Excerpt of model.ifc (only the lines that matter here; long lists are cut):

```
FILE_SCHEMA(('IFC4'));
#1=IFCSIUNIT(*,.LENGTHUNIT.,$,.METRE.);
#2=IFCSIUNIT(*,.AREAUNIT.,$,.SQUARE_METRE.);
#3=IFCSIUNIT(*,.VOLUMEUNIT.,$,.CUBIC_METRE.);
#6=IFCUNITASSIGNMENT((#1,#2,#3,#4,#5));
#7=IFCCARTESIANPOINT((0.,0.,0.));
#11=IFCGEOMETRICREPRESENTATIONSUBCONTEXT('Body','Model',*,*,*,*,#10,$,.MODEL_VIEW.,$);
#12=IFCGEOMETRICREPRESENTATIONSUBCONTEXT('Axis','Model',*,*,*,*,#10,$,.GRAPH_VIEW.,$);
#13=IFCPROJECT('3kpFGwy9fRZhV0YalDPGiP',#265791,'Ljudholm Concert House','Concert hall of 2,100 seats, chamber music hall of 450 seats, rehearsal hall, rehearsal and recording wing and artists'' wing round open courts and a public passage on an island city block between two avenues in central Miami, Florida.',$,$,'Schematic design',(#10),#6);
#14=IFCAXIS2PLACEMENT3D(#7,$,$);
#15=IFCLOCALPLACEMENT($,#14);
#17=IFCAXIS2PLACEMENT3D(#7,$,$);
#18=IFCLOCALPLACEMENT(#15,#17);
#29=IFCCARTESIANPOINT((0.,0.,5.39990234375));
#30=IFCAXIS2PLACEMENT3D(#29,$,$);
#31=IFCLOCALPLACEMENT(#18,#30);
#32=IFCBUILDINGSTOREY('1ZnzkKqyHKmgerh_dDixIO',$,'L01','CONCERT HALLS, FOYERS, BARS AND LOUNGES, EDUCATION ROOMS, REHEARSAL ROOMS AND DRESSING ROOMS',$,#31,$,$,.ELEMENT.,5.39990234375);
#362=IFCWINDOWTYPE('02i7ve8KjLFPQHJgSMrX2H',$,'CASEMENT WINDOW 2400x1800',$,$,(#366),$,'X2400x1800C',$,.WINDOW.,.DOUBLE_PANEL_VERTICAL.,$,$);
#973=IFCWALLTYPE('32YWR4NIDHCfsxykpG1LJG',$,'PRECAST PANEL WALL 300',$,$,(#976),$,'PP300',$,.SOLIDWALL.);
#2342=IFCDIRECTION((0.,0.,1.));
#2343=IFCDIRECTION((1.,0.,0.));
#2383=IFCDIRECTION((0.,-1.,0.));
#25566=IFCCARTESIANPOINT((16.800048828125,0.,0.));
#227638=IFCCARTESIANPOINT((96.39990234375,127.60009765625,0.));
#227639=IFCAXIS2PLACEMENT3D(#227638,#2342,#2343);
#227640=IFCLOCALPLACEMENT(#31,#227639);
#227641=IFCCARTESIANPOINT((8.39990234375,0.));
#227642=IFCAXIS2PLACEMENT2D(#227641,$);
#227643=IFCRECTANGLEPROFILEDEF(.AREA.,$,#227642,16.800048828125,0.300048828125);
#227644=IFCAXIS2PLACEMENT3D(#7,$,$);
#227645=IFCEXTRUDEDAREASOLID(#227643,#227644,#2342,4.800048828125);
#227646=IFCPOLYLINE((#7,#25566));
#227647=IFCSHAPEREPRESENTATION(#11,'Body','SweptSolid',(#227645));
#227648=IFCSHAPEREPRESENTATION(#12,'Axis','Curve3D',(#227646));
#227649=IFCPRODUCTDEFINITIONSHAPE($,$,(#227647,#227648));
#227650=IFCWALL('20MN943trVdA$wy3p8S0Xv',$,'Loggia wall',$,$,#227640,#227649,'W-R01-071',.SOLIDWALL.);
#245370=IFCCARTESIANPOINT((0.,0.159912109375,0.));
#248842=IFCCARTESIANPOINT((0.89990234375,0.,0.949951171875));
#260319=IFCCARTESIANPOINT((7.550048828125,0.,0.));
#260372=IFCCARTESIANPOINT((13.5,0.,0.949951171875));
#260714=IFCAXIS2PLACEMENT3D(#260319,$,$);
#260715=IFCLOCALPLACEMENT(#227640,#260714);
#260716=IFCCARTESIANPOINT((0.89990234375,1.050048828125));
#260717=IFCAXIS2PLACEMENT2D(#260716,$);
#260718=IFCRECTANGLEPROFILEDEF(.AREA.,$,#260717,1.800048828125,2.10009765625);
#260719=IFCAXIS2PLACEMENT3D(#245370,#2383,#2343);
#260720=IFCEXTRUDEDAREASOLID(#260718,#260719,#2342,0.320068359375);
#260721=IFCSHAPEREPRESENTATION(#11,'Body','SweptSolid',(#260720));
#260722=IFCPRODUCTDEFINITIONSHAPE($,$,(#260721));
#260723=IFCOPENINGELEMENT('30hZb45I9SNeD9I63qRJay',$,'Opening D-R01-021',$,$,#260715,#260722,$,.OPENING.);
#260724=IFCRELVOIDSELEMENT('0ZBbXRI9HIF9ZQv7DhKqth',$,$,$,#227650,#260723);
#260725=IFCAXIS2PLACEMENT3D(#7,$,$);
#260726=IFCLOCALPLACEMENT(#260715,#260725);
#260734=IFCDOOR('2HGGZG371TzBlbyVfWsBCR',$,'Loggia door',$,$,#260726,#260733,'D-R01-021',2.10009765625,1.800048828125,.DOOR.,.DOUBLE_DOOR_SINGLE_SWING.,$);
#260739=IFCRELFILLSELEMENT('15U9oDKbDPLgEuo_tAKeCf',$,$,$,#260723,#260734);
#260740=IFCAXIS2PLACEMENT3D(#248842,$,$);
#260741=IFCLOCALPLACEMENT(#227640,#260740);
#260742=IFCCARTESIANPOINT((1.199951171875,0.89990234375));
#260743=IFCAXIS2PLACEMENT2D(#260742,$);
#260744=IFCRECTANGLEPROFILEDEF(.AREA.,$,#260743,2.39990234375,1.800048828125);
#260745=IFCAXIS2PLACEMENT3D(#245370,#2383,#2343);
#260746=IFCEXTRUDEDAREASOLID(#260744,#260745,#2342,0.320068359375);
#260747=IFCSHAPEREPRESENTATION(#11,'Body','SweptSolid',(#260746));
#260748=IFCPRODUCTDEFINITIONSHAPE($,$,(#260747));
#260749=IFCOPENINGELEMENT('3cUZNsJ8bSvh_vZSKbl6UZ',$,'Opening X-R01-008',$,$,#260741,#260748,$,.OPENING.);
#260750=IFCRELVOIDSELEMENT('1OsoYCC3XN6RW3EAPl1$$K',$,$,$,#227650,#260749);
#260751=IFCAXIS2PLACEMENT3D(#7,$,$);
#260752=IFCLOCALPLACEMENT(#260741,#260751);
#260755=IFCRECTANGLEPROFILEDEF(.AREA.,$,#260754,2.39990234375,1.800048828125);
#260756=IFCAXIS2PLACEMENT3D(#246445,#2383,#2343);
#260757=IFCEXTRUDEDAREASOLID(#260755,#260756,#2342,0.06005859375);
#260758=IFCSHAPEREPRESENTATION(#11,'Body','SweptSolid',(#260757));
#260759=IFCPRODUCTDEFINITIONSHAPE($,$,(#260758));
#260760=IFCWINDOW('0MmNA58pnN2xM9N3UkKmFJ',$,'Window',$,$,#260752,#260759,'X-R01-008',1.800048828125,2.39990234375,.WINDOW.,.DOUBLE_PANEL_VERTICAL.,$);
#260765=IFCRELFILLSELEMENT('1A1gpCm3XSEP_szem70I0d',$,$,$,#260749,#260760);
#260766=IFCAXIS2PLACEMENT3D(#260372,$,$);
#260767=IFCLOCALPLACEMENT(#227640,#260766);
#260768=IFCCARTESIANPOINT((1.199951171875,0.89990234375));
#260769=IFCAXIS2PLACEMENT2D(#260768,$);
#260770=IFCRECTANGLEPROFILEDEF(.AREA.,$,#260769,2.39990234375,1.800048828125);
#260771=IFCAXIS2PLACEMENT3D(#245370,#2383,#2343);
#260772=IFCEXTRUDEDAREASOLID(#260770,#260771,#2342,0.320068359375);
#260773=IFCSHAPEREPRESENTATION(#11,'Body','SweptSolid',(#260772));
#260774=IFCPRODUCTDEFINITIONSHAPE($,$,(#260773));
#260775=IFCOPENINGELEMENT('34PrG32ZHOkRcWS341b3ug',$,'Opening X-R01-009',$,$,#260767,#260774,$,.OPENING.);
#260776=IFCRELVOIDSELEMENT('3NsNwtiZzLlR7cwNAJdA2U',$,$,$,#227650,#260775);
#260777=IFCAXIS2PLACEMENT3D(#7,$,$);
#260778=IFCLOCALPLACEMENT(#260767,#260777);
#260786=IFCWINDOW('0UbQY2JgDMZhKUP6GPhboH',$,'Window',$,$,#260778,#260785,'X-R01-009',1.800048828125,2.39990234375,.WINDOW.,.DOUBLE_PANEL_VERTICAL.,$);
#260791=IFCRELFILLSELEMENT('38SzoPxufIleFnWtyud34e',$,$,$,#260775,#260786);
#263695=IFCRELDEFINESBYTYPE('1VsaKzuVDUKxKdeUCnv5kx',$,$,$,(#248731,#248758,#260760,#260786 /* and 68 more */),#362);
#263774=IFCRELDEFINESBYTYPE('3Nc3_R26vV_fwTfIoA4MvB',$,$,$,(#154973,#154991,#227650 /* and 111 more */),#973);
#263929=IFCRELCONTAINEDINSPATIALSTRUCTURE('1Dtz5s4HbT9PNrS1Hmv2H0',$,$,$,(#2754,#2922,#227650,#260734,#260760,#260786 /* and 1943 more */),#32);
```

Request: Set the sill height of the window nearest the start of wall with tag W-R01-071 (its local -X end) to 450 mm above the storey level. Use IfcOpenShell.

```python
import numpy as np
import ifcopenshell
import ifcopenshell.api.geometry
import ifcopenshell.geom
import ifcopenshell.util.element
import ifcopenshell.util.placement
import ifcopenshell.util.shape
import ifcopenshell.util.unit

model = ifcopenshell.open("model.ifc")
unit_scale = ifcopenshell.util.unit.calculate_unit_scale(model)

window = model.by_guid("0MmNA58pnN2xM9N3UkKmFJ")
opening = window.FillsVoids[0].RelatingOpeningElement
storey = ifcopenshell.util.element.get_container(window, ifc_class="IfcBuildingStorey")
level = ifcopenshell.util.placement.get_local_placement(storey.ObjectPlacement)[2, 3]

# The opening's origin need not be at the sill, so measure its lowest point.
shape = ifcopenshell.geom.create_shape(ifcopenshell.geom.settings(), opening)
bottom = ifcopenshell.util.shape.get_shape_bottom_elevation(shape, shape.geometry) / unit_scale
dz = level + 0.45 - bottom

shift = np.array([0.0, 0.0, dz])
# The window is placed relative to its opening, so it follows when the opening moves.
matrix = ifcopenshell.util.placement.get_local_placement(opening.ObjectPlacement)
matrix[:3, 3] += shift
ifcopenshell.api.geometry.edit_object_placement(
    model, product=opening, matrix=matrix, is_si=False, should_transform_children=True
)

print(f"moved by {dz * unit_scale:+.3f} m")

model.write("model_v2.ifc")
```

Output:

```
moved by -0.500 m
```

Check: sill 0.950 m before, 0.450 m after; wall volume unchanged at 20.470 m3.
